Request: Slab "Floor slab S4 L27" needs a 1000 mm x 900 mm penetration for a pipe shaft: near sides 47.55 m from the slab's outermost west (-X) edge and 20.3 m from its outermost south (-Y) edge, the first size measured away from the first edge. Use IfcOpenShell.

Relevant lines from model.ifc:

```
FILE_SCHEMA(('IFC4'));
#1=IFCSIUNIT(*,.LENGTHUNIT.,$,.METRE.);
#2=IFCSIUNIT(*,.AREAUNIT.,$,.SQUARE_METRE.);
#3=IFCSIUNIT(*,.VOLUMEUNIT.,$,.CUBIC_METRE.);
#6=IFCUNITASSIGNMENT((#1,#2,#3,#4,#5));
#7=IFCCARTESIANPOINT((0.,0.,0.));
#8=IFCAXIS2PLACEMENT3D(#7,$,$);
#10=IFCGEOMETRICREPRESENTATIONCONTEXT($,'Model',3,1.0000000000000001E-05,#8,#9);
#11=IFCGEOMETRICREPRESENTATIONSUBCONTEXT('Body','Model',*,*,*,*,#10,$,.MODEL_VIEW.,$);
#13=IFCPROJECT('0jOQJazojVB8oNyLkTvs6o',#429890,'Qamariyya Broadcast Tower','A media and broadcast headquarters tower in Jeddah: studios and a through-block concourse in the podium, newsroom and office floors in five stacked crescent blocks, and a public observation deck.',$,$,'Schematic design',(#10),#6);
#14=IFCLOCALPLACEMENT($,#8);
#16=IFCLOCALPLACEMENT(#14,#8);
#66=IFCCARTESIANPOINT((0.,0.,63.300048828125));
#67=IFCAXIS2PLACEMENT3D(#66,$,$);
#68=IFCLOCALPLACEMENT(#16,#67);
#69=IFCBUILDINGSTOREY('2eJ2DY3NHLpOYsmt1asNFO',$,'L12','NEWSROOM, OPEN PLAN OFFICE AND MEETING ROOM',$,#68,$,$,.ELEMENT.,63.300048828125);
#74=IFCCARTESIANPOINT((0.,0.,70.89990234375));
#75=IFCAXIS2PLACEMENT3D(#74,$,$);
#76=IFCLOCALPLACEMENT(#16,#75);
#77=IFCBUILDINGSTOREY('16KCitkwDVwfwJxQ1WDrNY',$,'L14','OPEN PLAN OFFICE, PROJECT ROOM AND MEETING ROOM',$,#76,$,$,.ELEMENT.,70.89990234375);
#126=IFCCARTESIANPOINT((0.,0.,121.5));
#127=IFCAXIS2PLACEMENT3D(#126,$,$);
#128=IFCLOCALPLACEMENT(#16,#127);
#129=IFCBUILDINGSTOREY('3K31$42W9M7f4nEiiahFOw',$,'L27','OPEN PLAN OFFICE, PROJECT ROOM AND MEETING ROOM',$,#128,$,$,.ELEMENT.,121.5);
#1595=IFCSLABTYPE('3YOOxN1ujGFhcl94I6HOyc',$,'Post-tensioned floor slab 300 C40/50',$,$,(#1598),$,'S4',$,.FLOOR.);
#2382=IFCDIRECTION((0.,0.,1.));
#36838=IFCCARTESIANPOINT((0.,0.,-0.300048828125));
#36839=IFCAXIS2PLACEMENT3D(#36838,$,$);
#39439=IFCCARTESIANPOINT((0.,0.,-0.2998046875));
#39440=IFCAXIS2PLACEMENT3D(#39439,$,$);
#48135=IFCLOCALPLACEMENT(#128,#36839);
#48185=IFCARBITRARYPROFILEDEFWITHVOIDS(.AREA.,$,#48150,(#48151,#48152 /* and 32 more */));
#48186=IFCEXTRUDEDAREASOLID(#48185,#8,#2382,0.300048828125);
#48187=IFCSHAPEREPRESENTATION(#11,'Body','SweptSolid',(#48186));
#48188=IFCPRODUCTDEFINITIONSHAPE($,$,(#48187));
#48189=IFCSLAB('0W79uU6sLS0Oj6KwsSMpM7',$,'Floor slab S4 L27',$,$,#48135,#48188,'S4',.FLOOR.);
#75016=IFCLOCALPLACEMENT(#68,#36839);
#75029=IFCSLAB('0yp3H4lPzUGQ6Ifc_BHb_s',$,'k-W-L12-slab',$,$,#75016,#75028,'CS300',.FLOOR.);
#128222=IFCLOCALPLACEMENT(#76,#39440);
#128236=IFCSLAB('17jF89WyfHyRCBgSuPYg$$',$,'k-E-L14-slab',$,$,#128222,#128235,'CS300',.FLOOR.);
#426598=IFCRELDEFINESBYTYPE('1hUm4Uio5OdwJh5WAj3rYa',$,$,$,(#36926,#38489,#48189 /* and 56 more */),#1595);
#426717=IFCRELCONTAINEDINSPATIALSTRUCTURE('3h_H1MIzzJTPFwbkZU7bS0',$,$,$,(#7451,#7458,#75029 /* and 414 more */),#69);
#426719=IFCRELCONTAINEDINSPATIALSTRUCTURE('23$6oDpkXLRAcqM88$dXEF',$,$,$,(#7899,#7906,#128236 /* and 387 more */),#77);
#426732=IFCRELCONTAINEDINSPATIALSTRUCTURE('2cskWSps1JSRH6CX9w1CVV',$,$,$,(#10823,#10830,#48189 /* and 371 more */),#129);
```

```python
import numpy as np
import ifcopenshell
import ifcopenshell.api.feature
import ifcopenshell.api.geometry
import ifcopenshell.api.root
import ifcopenshell.geom
import ifcopenshell.util.placement
import ifcopenshell.util.representation
import ifcopenshell.util.shape
import ifcopenshell.util.unit

model = ifcopenshell.open("model.ifc")
unit_scale = ifcopenshell.util.unit.calculate_unit_scale(model)
settings = ifcopenshell.geom.settings()


def volume(element):
    """Net volume in cubic metres, openings subtracted."""
    shape = ifcopenshell.geom.create_shape(settings, element)
    return ifcopenshell.util.shape.get_volume(shape.geometry)


slab = model.by_guid("0W79uU6sLS0Oj6KwsSMpM7")
before = volume(slab)

# Extent in the slab's own axes, in metres. The edges named are its -X and -Y sides.
slab_shape = ifcopenshell.geom.create_shape(settings, slab)
vertices = ifcopenshell.util.shape.get_vertices(slab_shape.geometry)
x_min, y_min, bottom = vertices.min(axis=0)
top = vertices[:, 2].max()

opening = ifcopenshell.api.root.create_entity(model, ifc_class="IfcOpeningElement", name="Pipe shaft opening", predefined_type="OPENING")
context = ifcopenshell.util.representation.get_context(model, "Model", "Body", "MODEL_VIEW")
width, depth = 1, 0.9
outline = [(0.0, 0.0), (width, 0.0), (width, depth), (0.0, depth), (0.0, 0.0)]
# Overshoot both faces by 50 mm so the cut is clean.
shape = ifcopenshell.api.geometry.add_slab_representation(
    model, context=context, depth=top - bottom + 0.1, polyline=outline
)
ifcopenshell.api.geometry.assign_representation(model, product=opening, representation=shape)

matrix = ifcopenshell.util.placement.get_local_placement(slab.ObjectPlacement)
matrix[:, 3] = matrix @ np.append(np.array([x_min + 47.55, y_min + 20.3, bottom - 0.05]) / unit_scale, 1.0)
ifcopenshell.api.geometry.edit_object_placement(model, product=opening, matrix=matrix, is_si=False)
ifcopenshell.api.feature.add_feature(model, feature=opening, element=slab)

after = volume(slab)

print(f"slab volume {before:.3f} -> {after:.3f} m3")

model.write("model_rev.ifc")
```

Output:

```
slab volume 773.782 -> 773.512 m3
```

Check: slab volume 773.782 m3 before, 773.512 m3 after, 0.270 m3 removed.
